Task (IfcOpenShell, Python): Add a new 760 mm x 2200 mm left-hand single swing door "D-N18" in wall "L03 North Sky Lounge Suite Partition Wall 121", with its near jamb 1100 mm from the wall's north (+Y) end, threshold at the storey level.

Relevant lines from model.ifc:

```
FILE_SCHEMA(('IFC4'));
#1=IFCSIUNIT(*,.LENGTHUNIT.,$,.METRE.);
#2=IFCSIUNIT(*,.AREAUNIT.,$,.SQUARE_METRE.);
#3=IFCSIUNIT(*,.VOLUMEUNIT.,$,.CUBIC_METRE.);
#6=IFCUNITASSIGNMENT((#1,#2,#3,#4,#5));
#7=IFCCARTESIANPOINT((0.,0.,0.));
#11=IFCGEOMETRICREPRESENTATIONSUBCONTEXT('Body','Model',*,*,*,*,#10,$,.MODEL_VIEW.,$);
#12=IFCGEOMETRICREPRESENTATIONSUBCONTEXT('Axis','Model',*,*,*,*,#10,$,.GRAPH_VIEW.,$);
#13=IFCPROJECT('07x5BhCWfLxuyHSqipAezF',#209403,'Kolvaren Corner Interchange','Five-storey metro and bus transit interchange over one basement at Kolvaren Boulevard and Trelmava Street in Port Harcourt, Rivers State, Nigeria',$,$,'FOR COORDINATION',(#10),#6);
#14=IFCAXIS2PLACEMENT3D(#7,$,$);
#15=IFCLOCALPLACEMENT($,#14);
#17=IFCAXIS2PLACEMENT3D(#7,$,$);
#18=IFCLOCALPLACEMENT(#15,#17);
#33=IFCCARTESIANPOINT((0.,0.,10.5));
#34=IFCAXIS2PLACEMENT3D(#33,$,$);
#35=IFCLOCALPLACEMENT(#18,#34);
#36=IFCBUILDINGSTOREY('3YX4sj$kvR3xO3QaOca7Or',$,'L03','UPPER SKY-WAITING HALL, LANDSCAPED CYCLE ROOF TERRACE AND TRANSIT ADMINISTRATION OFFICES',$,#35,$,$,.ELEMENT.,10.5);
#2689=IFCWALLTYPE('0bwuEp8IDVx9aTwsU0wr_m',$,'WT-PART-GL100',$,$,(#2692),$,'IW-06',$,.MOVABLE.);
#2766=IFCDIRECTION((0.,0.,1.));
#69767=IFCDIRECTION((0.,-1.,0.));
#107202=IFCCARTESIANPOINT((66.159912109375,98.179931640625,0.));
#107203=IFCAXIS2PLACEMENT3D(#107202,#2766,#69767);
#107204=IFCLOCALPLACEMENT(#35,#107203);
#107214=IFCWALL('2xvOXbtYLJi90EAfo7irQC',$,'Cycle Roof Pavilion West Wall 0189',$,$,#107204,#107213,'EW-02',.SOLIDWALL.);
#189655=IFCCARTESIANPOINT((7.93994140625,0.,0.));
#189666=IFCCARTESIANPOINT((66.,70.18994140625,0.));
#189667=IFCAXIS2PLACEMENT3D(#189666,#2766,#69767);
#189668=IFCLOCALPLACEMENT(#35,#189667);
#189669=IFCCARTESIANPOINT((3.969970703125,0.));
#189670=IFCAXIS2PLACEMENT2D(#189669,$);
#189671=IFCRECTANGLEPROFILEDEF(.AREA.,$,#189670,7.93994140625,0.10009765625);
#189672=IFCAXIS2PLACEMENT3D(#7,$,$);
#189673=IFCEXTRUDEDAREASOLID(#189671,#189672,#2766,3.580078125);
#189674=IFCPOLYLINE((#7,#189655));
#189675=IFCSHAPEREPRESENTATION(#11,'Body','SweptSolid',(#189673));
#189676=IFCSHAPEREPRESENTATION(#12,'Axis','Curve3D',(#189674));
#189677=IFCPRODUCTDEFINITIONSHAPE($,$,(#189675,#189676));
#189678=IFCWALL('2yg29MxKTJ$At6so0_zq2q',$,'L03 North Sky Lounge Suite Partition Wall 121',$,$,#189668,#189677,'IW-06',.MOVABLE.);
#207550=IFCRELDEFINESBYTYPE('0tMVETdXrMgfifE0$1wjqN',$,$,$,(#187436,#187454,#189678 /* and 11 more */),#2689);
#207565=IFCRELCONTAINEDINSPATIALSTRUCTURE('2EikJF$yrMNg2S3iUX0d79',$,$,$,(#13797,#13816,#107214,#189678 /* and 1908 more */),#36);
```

```python
import numpy as np
import ifcopenshell
import ifcopenshell.api.feature
import ifcopenshell.api.geometry
import ifcopenshell.api.root
import ifcopenshell.api.spatial
import ifcopenshell.geom
import ifcopenshell.util.element
import ifcopenshell.util.placement
import ifcopenshell.util.representation
import ifcopenshell.util.shape
import ifcopenshell.util.unit

model = ifcopenshell.open("model.ifc")
unit_scale = ifcopenshell.util.unit.calculate_unit_scale(model)
settings = ifcopenshell.geom.settings()


def volume(element):
    """Net volume in cubic metres, openings subtracted."""
    shape = ifcopenshell.geom.create_shape(settings, element)
    return ifcopenshell.util.shape.get_volume(shape.geometry)


wall = model.by_id(189678)
storey = ifcopenshell.util.element.get_container(wall, ifc_class="IfcBuildingStorey")
context = ifcopenshell.util.representation.get_context(model, "Model", "Body", "MODEL_VIEW")
before = volume(wall)

width, height, from_end, sill = 0.76, 2.2, 1.1, 0.0  # metres

# The wall runs along its own X axis, and the end named is its -X end.
wall_shape = ifcopenshell.geom.create_shape(settings, wall)
x, y, z = ifcopenshell.util.shape.get_vertices(wall_shape.geometry).T
start = x.min() + from_end
face, thickness = float(y.min()), float(y.max() - y.min())
wall_matrix = ifcopenshell.util.placement.get_local_placement(wall.ObjectPlacement)
level = ifcopenshell.util.placement.get_local_placement(storey.ObjectPlacement)[2, 3]


def in_wall(x, y):
    """Placement at x, y metres in the wall's axes, at sill height."""
    matrix = wall_matrix.copy()
    matrix[:, 3] = wall_matrix @ np.array([x / unit_scale, y / unit_scale, 0.0, 1.0])
    matrix[2, 3] = level + sill / unit_scale
    return matrix


# Opening: a box that overshoots both wall faces by 50 mm.
opening = ifcopenshell.api.root.create_entity(model, ifc_class="IfcOpeningElement", predefined_type="OPENING")
box = ifcopenshell.api.geometry.add_wall_representation(
    model, context=context, length=width, height=height, thickness=thickness + 0.1
)
ifcopenshell.api.geometry.assign_representation(model, product=opening, representation=box)
ifcopenshell.api.geometry.edit_object_placement(model, product=opening, matrix=in_wall(start, face - 0.05), is_si=False)
ifcopenshell.api.feature.add_feature(model, feature=opening, element=wall)

door = ifcopenshell.api.root.create_entity(model, ifc_class="IfcDoor", name="D-N18", predefined_type="DOOR")
door.OverallWidth, door.OverallHeight = width / unit_scale, height / unit_scale
door.OperationType = "SINGLE_SWING_LEFT"
body = ifcopenshell.api.geometry.add_door_representation(
    model,
    context=context,
    overall_width=door.OverallWidth,
    overall_height=door.OverallHeight,
    operation_type="SINGLE_SWING_LEFT",
    lining_properties={"LiningDepth": thickness / unit_scale, "ThresholdDepth": thickness / unit_scale},
)
ifcopenshell.api.geometry.assign_representation(model, product=door, representation=body)
ifcopenshell.api.spatial.assign_container(model, products=[door], relating_structure=storey)
ifcopenshell.api.feature.add_filling(model, opening=opening, element=door)

# The lining spans the wall, so the door starts at the wall face.
ifcopenshell.api.geometry.edit_object_placement(model, product=door, matrix=in_wall(start, face), is_si=False)

after = volume(wall)

print(f"wall volume {before:.3f} -> {after:.3f} m3")

model.write("model_edited.ifc")
```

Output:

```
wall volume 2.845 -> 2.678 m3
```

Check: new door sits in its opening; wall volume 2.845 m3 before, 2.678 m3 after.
